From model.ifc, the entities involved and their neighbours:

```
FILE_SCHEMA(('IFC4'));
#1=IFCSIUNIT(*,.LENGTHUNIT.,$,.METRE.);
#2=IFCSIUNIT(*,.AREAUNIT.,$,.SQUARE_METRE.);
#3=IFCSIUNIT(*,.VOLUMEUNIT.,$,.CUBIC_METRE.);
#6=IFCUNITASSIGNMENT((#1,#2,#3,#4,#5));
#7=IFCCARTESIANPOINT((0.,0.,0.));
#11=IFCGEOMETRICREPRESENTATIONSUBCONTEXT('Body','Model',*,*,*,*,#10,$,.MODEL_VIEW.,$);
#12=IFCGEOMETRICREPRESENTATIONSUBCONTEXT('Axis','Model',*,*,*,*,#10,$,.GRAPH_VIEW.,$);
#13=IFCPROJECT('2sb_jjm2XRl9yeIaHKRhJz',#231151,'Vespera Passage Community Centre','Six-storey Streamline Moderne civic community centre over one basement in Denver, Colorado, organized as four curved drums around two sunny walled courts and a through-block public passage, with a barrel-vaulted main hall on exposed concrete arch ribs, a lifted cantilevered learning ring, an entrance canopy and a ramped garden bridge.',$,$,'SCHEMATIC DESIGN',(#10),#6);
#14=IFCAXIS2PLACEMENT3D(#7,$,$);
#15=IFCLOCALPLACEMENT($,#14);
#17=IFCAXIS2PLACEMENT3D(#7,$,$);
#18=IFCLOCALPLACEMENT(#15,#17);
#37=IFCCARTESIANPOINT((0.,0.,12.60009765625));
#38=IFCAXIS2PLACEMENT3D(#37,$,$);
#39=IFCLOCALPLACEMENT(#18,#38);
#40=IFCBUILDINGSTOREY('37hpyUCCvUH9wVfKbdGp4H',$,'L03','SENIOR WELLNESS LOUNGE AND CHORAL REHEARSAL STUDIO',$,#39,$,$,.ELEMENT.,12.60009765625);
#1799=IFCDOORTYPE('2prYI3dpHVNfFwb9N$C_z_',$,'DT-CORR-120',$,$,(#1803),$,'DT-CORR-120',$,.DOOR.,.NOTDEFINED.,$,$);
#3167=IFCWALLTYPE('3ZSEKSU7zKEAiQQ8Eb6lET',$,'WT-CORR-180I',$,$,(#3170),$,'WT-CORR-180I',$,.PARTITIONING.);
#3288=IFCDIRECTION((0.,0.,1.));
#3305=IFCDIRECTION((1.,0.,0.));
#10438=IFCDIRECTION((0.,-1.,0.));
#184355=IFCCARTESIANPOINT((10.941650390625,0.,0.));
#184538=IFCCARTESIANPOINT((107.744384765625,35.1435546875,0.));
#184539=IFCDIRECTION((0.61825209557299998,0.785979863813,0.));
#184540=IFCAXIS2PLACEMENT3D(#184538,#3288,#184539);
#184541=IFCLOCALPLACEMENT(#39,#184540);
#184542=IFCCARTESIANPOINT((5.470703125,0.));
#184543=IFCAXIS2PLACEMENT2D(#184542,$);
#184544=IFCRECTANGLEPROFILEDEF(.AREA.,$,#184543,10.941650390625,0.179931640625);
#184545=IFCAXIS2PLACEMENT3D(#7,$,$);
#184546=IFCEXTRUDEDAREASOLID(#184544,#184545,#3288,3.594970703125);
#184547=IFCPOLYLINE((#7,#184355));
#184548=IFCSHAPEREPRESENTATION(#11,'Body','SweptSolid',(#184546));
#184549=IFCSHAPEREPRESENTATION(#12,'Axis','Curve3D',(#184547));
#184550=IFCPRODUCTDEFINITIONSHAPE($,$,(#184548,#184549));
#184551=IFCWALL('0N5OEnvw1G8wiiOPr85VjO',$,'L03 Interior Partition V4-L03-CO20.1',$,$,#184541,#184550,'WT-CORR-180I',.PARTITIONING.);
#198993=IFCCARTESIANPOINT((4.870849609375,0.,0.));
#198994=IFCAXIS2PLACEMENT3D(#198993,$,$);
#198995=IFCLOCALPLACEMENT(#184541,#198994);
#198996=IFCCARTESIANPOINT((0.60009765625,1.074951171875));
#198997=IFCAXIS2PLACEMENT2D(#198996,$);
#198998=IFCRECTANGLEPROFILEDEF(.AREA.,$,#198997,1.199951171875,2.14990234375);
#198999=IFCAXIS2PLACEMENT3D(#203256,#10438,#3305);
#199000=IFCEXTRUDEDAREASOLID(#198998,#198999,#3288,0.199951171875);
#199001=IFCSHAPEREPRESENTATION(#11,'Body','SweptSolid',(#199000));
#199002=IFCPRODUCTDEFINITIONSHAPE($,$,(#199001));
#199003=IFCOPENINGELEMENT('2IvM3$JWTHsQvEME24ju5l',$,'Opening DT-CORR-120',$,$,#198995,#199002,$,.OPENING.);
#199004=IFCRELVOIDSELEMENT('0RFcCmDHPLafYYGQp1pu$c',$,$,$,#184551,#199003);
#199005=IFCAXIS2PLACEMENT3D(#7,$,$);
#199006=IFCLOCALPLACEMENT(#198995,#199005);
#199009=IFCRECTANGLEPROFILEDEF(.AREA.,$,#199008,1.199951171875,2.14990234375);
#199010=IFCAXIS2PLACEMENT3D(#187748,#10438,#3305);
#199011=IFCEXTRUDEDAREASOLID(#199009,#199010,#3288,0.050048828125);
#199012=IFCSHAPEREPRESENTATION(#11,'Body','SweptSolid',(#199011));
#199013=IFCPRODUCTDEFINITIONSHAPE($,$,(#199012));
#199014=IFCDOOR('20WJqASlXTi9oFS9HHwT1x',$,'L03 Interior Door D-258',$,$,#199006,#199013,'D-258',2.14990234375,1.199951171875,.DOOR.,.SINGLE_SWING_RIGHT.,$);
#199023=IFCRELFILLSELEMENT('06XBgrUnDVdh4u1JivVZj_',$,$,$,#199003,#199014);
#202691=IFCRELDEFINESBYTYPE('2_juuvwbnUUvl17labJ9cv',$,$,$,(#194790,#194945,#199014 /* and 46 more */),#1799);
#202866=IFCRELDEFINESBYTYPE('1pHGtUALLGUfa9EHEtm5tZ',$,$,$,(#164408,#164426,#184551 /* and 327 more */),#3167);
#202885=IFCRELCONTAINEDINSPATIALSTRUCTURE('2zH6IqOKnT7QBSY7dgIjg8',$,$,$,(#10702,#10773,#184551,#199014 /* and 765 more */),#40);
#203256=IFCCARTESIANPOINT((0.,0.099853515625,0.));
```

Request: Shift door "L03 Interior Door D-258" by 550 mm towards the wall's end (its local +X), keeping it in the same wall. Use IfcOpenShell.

```python
import ifcopenshell
import ifcopenshell.api.geometry
import ifcopenshell.util.placement
import ifcopenshell.util.unit

model = ifcopenshell.open("model.ifc")
unit_scale = ifcopenshell.util.unit.calculate_unit_scale(model)

door = model.by_id(199014)
opening = door.FillsVoids[0].RelatingOpeningElement
wall = opening.VoidsElements[0].RelatingBuildingElement

wall_matrix = ifcopenshell.util.placement.get_local_placement(wall.ObjectPlacement)
shift = wall_matrix[:3, 0] * 0.55 / unit_scale
before = ifcopenshell.util.placement.get_local_placement(door.ObjectPlacement)[:3, 3].copy()

# The door is placed relative to its opening, so it follows when the opening moves.
matrix = ifcopenshell.util.placement.get_local_placement(opening.ObjectPlacement)
matrix[:3, 3] += shift
ifcopenshell.api.geometry.edit_object_placement(
    model, product=opening, matrix=matrix, is_si=False, should_transform_children=True
)

after = ifcopenshell.util.placement.get_local_placement(door.ObjectPlacement)[:3, 3]
print("door moved by", (after - before).round(3) + 0.0)

model.write("model-out.ifc")
```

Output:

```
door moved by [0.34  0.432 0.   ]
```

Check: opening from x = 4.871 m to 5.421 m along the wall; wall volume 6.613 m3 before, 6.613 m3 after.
